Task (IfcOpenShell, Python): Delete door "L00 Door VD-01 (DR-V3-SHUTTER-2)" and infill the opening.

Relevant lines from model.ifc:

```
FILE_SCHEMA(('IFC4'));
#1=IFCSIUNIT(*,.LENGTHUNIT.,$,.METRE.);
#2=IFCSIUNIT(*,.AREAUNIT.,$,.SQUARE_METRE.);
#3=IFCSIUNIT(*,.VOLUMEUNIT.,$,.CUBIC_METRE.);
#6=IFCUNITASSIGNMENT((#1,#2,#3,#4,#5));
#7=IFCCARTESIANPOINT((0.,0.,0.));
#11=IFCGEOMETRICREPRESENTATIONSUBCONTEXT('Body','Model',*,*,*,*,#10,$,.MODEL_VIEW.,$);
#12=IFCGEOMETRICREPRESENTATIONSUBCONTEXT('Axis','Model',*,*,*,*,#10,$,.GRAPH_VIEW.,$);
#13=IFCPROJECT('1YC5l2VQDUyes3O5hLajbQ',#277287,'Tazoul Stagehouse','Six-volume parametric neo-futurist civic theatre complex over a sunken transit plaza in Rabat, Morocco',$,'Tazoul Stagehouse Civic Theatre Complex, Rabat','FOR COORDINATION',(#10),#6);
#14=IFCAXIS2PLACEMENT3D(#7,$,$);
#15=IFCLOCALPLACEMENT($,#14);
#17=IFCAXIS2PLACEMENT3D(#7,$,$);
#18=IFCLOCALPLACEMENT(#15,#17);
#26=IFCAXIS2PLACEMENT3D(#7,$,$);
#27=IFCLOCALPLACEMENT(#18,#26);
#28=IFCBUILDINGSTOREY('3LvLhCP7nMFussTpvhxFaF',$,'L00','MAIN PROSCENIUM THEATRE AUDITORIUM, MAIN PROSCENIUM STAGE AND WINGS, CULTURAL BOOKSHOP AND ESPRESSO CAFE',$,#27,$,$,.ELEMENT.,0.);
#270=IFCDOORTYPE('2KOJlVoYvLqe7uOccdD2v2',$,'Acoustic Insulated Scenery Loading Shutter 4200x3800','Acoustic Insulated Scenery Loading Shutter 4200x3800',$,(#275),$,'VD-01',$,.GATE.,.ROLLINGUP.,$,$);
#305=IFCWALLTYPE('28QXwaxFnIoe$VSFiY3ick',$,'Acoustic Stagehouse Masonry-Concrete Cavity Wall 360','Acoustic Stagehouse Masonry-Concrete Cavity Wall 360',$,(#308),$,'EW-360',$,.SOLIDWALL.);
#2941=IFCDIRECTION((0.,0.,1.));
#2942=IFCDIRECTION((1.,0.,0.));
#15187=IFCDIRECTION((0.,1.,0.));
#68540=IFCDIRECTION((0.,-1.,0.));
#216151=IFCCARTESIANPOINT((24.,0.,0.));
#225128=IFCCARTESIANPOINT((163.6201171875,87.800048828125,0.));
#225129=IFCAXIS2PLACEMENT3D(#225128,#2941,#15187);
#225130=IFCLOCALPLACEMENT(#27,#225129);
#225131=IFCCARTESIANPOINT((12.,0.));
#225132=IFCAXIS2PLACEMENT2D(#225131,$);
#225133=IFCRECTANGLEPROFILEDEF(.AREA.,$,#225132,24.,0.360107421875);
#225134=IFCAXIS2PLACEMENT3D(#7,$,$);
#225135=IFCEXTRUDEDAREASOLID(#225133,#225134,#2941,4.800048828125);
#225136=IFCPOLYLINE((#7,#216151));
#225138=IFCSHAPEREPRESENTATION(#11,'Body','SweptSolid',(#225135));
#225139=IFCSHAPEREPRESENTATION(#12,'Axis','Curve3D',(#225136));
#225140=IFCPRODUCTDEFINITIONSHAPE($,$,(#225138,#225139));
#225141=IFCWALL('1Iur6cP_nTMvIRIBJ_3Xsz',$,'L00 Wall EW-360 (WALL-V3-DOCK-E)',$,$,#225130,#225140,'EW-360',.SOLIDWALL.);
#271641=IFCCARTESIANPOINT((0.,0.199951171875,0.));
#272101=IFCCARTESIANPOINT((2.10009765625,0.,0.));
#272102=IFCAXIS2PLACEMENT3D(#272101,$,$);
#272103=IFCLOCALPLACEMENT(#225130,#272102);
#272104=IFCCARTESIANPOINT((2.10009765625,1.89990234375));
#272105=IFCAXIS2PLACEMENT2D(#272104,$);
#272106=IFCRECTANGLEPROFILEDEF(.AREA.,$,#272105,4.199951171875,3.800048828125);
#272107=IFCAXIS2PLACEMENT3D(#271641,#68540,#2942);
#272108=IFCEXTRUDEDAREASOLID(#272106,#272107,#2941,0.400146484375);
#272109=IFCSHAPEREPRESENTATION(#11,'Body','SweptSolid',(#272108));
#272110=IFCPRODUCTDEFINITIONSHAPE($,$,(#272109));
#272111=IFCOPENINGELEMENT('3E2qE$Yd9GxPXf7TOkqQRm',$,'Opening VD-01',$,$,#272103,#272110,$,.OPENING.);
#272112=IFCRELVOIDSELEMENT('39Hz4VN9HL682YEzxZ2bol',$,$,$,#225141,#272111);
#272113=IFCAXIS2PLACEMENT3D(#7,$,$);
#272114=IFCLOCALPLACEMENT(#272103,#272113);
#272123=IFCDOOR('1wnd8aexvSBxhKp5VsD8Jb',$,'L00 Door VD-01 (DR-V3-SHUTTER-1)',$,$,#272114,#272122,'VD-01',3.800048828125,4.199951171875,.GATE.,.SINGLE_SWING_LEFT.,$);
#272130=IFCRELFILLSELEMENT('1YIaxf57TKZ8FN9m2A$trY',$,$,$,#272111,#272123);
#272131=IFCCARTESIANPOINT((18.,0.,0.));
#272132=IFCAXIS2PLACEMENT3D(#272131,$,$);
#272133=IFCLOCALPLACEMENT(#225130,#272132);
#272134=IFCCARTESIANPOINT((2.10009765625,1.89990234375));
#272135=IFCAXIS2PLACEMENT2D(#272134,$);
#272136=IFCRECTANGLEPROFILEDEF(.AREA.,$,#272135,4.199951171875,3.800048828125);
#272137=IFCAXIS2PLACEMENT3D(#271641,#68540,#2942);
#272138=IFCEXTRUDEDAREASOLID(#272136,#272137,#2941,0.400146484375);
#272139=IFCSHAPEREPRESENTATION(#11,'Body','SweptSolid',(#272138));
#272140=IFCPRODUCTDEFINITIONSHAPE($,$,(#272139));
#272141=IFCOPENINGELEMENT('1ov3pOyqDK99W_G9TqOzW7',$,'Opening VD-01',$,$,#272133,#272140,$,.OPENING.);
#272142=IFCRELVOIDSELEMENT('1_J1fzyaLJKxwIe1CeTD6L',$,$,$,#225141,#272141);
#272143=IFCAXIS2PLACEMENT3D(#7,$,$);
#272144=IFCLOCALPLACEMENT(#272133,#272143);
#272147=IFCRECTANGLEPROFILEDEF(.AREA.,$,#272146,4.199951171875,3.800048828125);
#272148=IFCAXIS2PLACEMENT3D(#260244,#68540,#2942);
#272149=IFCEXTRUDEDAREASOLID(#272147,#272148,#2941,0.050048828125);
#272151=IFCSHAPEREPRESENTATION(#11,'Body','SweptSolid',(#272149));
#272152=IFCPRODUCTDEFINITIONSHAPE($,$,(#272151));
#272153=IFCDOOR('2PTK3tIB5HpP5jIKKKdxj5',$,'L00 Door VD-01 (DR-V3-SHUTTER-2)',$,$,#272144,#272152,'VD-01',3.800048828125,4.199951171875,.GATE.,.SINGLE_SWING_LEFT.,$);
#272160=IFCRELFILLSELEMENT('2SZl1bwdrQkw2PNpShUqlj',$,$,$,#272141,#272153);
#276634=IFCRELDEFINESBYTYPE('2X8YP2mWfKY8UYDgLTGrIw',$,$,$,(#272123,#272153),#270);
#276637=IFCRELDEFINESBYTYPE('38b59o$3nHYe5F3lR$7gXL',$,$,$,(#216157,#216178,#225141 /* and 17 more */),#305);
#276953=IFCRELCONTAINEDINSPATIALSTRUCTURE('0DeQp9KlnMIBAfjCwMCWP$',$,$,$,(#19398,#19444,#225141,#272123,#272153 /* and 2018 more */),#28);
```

```python
import ifcopenshell
import ifcopenshell.api.feature
import ifcopenshell.api.root
import ifcopenshell.geom
import ifcopenshell.util.shape

model = ifcopenshell.open("model.ifc")
settings = ifcopenshell.geom.settings()


def volume(element):
    """Net volume in cubic metres, openings subtracted."""
    shape = ifcopenshell.geom.create_shape(settings, element)
    return ifcopenshell.util.shape.get_volume(shape.geometry)


door = model.by_guid("2PTK3tIB5HpP5jIKKKdxj5")
opening = door.FillsVoids[0].RelatingOpeningElement
wall = opening.VoidsElements[0].RelatingBuildingElement
before = volume(wall)

ifcopenshell.api.root.remove_product(model, product=door)
ifcopenshell.api.feature.remove_feature(model, feature=opening)

after = volume(wall)

print(f"wall volume {before:.3f} -> {after:.3f} m3")

model.write("model-out.ifc")
```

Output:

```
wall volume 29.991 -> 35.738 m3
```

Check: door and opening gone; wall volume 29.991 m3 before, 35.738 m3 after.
